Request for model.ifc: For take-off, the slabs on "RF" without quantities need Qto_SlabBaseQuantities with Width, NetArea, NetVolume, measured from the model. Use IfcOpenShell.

First a look at what the model holds.

```python
import ifcopenshell
import ifcopenshell.util.element
import ifcopenshell.util.unit

model = ifcopenshell.open("model.ifc")
print(model.schema)
for unit_type in ("LENGTHUNIT", "AREAUNIT", "VOLUMEUNIT"):
    print(unit_type, ifcopenshell.util.unit.calculate_unit_scale(model, unit_type))
storey = next(s for s in model.by_type("IfcBuildingStorey") if s.Name == "RF")
slabs = [e for e in ifcopenshell.util.element.get_decomposition(storey) if e.is_a("IfcSlab")]
for e in sorted(slabs, key=lambda e: e.id()):
    print(e.id(), e.is_a(), e.Name, list(ifcopenshell.util.element.get_psets(e, qtos_only=True)), sep=" | ")
```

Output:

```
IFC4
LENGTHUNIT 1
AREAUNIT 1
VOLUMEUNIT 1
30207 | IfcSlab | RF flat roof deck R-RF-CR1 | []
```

```python
import ifcopenshell
import ifcopenshell.api.pset
import ifcopenshell.geom
import ifcopenshell.util.element
import ifcopenshell.util.shape
import ifcopenshell.util.unit

model = ifcopenshell.open("model.ifc")
unit_scale = ifcopenshell.util.unit.calculate_unit_scale(model)
area_scale = ifcopenshell.util.unit.calculate_unit_scale(model, "AREAUNIT")
volume_scale = ifcopenshell.util.unit.calculate_unit_scale(model, "VOLUMEUNIT")
settings = ifcopenshell.geom.settings()

storey = next(s for s in model.by_type("IfcBuildingStorey") if s.Name == "RF")
slabs = [e for e in ifcopenshell.util.element.get_decomposition(storey) if e.is_a("IfcSlab")]

for e in sorted(slabs, key=lambda e: e.id()):
    if ifcopenshell.util.element.get_psets(e, qtos_only=True, should_inherit=False):
        continue
    # Geometry comes back in metres, in the element's own axes.
    shape = ifcopenshell.geom.create_shape(settings, e)
    values = {
        "Width": ifcopenshell.util.shape.get_z(shape.geometry) / unit_scale,
        "NetArea": ifcopenshell.util.shape.get_footprint_area(shape.geometry) / area_scale,
        "NetVolume": ifcopenshell.util.shape.get_volume(shape.geometry) / volume_scale,
    }
    qto = ifcopenshell.api.pset.add_qto(model, product=e, name="Qto_SlabBaseQuantities")
    ifcopenshell.api.pset.edit_qto(model, qto=qto, properties=values)
    print(e.id(), {k: round(v, 3) for k, v in values.items()})

model.write("model-out.ifc")
```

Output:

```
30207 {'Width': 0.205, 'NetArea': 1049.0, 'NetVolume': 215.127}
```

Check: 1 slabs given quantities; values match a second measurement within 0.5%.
